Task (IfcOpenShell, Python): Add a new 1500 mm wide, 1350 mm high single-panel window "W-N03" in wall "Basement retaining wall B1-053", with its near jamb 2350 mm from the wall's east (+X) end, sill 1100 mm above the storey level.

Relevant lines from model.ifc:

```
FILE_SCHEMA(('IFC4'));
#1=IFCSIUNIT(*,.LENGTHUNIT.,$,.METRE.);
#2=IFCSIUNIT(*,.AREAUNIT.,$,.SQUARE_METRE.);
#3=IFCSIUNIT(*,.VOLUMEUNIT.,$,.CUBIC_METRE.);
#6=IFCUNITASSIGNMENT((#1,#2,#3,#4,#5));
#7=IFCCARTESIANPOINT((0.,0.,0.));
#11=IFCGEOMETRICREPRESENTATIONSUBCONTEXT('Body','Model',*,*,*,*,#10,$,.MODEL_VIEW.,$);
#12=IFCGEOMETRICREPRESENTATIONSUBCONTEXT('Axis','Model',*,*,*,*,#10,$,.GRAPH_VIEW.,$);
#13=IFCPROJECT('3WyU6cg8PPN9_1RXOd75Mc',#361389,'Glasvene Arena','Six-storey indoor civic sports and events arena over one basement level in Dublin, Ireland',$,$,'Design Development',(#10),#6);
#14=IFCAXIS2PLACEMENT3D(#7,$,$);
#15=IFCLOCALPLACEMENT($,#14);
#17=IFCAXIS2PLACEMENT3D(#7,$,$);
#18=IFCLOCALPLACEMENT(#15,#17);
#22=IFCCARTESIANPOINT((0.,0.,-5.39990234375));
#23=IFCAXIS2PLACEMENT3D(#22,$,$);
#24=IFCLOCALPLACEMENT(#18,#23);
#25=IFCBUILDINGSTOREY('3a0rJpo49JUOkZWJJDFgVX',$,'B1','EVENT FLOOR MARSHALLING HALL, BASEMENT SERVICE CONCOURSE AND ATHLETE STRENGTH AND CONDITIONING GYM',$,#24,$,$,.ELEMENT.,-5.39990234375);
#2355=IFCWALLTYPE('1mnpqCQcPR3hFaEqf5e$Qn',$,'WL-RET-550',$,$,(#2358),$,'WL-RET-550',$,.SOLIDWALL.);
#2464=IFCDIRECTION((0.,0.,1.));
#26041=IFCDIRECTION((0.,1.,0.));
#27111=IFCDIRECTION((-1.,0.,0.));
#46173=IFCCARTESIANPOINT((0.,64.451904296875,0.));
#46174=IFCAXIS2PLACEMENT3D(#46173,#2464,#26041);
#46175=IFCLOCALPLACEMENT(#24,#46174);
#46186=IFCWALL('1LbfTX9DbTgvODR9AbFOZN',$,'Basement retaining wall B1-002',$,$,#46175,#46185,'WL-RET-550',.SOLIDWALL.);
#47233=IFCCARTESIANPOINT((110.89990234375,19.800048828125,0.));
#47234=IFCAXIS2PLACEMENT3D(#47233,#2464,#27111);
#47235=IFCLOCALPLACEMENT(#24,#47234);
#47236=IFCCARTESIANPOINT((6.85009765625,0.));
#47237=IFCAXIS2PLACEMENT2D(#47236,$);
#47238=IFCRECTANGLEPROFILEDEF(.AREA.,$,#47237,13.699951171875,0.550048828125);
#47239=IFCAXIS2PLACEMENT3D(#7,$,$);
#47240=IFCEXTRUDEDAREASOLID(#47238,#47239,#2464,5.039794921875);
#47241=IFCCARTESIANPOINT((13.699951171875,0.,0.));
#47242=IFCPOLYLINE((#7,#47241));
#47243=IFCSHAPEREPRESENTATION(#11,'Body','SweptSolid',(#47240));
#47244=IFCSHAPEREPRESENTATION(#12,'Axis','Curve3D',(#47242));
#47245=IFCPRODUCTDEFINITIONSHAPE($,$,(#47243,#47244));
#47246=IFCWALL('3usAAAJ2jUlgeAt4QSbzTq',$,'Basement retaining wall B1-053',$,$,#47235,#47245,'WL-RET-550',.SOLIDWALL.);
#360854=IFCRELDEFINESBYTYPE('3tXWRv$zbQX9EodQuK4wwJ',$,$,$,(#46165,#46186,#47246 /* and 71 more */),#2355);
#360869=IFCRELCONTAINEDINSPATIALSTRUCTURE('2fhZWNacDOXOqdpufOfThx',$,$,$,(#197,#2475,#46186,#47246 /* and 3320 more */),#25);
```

```python
import numpy as np
import ifcopenshell
import ifcopenshell.api.feature
import ifcopenshell.api.geometry
import ifcopenshell.api.root
import ifcopenshell.api.spatial
import ifcopenshell.geom
import ifcopenshell.util.element
import ifcopenshell.util.placement
import ifcopenshell.util.representation
import ifcopenshell.util.shape
import ifcopenshell.util.unit

model = ifcopenshell.open("model.ifc")
unit_scale = ifcopenshell.util.unit.calculate_unit_scale(model)
settings = ifcopenshell.geom.settings()


def volume(element):
    """Net volume in cubic metres, openings subtracted."""
    shape = ifcopenshell.geom.create_shape(settings, element)
    return ifcopenshell.util.shape.get_volume(shape.geometry)


wall = model.by_guid("3usAAAJ2jUlgeAt4QSbzTq")
storey = ifcopenshell.util.element.get_container(wall, ifc_class="IfcBuildingStorey")
context = ifcopenshell.util.representation.get_context(model, "Model", "Body", "MODEL_VIEW")
before = volume(wall)

width, height, from_end, sill = 1.5, 1.35, 2.35, 1.1  # metres

# The wall runs along its own X axis, and the end named is its -X end.
wall_shape = ifcopenshell.geom.create_shape(settings, wall)
x, y, z = ifcopenshell.util.shape.get_vertices(wall_shape.geometry).T
start = x.min() + from_end
face, thickness = float(y.min()), float(y.max() - y.min())
wall_matrix = ifcopenshell.util.placement.get_local_placement(wall.ObjectPlacement)
level = ifcopenshell.util.placement.get_local_placement(storey.ObjectPlacement)[2, 3]


def in_wall(x, y):
    """Placement at x, y metres in the wall's axes, at sill height."""
    matrix = wall_matrix.copy()
    matrix[:, 3] = wall_matrix @ np.array([x / unit_scale, y / unit_scale, 0.0, 1.0])
    matrix[2, 3] = level + sill / unit_scale
    return matrix


# Opening: a box that overshoots both wall faces by 50 mm.
opening = ifcopenshell.api.root.create_entity(model, ifc_class="IfcOpeningElement", predefined_type="OPENING")
box = ifcopenshell.api.geometry.add_wall_representation(
    model, context=context, length=width, height=height, thickness=thickness + 0.1
)
ifcopenshell.api.geometry.assign_representation(model, product=opening, representation=box)
ifcopenshell.api.geometry.edit_object_placement(model, product=opening, matrix=in_wall(start, face - 0.05), is_si=False)
ifcopenshell.api.feature.add_feature(model, feature=opening, element=wall)

window = ifcopenshell.api.root.create_entity(model, ifc_class="IfcWindow", name="W-N03", predefined_type="WINDOW")
window.OverallWidth, window.OverallHeight = width / unit_scale, height / unit_scale
window.PartitioningType = "SINGLE_PANEL"
body = ifcopenshell.api.geometry.add_window_representation(
    model,
    context=context,
    overall_width=window.OverallWidth,
    overall_height=window.OverallHeight,
    partition_type="SINGLE_PANEL",
)
ifcopenshell.api.geometry.assign_representation(model, product=window, representation=body)
ifcopenshell.api.spatial.assign_container(model, products=[window], relating_structure=storey)
ifcopenshell.api.feature.add_filling(model, opening=opening, element=window)

# Centre the window in the wall's thickness.
ifcopenshell.api.geometry.edit_object_placement(model, product=window, matrix=in_wall(start, face), is_si=False)
window_shape = ifcopenshell.geom.create_shape(settings, window)
depth = ifcopenshell.util.shape.get_vertices(window_shape.geometry)[:, 1]
offset = face + thickness / 2 - (depth.min() + depth.max()) / 2
ifcopenshell.api.geometry.edit_object_placement(model, product=window, matrix=in_wall(start, offset), is_si=False)

after = volume(wall)

print(f"wall volume {before:.3f} -> {after:.3f} m3")

model.write("model_edited.ifc")
```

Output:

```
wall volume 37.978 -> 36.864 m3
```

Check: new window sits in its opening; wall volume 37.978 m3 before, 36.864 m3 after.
